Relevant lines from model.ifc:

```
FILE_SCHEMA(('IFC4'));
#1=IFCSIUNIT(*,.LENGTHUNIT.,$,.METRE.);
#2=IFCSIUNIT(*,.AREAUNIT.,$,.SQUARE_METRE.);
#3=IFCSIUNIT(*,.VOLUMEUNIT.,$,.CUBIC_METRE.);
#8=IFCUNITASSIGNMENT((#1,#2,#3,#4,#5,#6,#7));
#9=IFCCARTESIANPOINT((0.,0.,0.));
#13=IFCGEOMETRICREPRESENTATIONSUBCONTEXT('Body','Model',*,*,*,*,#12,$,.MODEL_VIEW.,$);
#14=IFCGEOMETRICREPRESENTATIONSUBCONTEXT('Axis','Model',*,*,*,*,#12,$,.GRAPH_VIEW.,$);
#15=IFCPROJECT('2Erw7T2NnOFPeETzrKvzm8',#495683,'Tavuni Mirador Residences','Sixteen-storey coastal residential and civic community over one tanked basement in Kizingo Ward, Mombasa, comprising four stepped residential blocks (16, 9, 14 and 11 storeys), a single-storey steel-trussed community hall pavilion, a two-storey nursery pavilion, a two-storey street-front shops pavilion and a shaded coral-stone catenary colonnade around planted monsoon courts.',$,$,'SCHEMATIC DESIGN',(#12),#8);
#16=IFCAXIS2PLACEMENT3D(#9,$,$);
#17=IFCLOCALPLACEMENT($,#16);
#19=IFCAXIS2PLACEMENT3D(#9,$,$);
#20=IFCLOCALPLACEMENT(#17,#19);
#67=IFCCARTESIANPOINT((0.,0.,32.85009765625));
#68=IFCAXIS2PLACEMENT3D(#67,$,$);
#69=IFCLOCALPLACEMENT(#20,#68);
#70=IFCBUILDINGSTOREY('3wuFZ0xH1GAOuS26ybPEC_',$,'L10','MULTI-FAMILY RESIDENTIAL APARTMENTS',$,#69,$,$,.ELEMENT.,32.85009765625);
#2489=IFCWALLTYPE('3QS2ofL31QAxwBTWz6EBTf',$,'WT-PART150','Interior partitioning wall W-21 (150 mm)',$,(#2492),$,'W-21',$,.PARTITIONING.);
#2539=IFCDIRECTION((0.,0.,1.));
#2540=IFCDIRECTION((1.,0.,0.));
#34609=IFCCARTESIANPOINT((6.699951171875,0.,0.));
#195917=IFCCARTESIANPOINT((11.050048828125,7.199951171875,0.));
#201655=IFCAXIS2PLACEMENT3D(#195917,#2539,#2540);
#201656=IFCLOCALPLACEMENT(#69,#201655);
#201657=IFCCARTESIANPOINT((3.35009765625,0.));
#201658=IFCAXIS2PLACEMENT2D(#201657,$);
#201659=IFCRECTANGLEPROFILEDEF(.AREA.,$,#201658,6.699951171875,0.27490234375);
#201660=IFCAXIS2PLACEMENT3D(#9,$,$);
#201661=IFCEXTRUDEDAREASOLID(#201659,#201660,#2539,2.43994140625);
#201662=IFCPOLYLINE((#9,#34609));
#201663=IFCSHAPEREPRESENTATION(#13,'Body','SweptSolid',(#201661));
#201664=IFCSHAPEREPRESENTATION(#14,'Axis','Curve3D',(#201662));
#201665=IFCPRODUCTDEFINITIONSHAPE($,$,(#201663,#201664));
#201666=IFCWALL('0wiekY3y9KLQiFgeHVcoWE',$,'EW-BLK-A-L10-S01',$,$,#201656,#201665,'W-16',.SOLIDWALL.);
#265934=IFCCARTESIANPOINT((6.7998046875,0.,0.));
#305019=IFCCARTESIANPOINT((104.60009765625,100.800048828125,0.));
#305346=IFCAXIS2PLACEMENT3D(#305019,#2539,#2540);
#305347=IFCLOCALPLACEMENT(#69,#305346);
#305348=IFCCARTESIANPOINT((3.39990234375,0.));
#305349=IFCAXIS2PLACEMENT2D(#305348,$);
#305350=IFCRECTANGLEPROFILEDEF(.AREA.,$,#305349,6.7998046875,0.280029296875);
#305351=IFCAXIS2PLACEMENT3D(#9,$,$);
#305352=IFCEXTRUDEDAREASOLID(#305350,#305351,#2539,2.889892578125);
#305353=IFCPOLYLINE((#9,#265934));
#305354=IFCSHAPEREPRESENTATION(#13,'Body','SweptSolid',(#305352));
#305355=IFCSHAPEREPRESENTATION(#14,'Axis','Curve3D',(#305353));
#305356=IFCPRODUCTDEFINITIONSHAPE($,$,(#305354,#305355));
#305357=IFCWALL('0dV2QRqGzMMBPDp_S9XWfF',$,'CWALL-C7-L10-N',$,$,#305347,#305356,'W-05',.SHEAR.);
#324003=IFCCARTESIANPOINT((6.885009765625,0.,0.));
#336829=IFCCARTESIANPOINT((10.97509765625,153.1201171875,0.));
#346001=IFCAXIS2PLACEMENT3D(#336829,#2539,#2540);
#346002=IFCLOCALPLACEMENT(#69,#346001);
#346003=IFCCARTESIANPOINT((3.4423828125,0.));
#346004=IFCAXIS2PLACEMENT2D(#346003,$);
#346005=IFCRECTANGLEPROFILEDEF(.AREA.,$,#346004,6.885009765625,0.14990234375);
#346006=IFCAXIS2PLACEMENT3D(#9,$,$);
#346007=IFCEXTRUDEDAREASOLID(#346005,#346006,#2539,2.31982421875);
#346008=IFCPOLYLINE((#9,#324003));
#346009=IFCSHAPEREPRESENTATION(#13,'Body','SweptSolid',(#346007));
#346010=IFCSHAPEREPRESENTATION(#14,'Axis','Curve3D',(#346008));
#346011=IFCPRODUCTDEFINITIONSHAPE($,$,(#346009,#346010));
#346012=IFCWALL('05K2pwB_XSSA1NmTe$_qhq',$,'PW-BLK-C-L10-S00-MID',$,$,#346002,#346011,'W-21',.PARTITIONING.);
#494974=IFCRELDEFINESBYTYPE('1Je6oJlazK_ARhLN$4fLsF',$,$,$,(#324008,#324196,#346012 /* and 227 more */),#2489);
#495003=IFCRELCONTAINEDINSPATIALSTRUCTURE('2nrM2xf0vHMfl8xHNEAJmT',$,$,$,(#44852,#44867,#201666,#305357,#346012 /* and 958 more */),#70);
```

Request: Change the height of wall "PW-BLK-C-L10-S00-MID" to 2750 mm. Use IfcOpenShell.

```python
import ifcopenshell
import ifcopenshell.geom
import ifcopenshell.util.representation
import ifcopenshell.util.shape

model = ifcopenshell.open("model.ifc")
settings = ifcopenshell.geom.settings()


def volume(element):
    """Net volume in cubic metres, openings subtracted."""
    shape = ifcopenshell.geom.create_shape(settings, element)
    return ifcopenshell.util.shape.get_volume(shape.geometry)


wall = model.by_guid("05K2pwB_XSSA1NmTe$_qhq")
before = volume(wall)

body = ifcopenshell.util.representation.get_representation(wall, "Model", "Body")
solid = body.Items[0]
old_height = solid.Depth
solid.Depth = 2.75
after = volume(wall)

print(f"height {old_height:g} -> {solid.Depth:g}, volume {before:.3f} -> {after:.3f} m3")

model.write("model_rev.ifc")
```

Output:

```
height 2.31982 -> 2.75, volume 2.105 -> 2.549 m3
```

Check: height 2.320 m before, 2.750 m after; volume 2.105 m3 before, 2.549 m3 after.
